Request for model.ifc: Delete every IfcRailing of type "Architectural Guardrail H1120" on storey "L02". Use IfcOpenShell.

First a look at what the model holds.

```python
import ifcopenshell
import ifcopenshell.util.element

model = ifcopenshell.open("model.ifc")
print(model.schema)
storey = next(s for s in model.by_type("IfcBuildingStorey") if s.Name == "L02")
railings = [e for e in ifcopenshell.util.element.get_decomposition(storey) if e.is_a("IfcRailing")]
seen = {}
for e in railings:
    element_type = ifcopenshell.util.element.get_type(e)
    name = element_type.Name if element_type not in (None, e) else None
    seen[name] = seen.get(name, 0) + 1
for name, count in sorted(seen.items(), key=str):
    print(count, "x", name)
```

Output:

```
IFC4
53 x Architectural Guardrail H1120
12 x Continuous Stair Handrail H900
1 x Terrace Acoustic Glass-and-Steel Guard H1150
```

```python
import ifcopenshell
import ifcopenshell.api.root
import ifcopenshell.util.element

model = ifcopenshell.open("model.ifc")

storey = next(s for s in model.by_type("IfcBuildingStorey") if s.Name == "L02")
railings = [e for e in ifcopenshell.util.element.get_decomposition(storey) if e.is_a("IfcRailing")]
targets = [e for e in railings if (t := ifcopenshell.util.element.get_type(e)) not in (None, e) and t.Name == "Architectural Guardrail H1120"]

for e in targets:
    ifcopenshell.api.root.remove_product(model, product=e)
print(len(targets), "removed")

model.write("model_rev.ifc")
```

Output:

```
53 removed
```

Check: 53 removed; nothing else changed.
